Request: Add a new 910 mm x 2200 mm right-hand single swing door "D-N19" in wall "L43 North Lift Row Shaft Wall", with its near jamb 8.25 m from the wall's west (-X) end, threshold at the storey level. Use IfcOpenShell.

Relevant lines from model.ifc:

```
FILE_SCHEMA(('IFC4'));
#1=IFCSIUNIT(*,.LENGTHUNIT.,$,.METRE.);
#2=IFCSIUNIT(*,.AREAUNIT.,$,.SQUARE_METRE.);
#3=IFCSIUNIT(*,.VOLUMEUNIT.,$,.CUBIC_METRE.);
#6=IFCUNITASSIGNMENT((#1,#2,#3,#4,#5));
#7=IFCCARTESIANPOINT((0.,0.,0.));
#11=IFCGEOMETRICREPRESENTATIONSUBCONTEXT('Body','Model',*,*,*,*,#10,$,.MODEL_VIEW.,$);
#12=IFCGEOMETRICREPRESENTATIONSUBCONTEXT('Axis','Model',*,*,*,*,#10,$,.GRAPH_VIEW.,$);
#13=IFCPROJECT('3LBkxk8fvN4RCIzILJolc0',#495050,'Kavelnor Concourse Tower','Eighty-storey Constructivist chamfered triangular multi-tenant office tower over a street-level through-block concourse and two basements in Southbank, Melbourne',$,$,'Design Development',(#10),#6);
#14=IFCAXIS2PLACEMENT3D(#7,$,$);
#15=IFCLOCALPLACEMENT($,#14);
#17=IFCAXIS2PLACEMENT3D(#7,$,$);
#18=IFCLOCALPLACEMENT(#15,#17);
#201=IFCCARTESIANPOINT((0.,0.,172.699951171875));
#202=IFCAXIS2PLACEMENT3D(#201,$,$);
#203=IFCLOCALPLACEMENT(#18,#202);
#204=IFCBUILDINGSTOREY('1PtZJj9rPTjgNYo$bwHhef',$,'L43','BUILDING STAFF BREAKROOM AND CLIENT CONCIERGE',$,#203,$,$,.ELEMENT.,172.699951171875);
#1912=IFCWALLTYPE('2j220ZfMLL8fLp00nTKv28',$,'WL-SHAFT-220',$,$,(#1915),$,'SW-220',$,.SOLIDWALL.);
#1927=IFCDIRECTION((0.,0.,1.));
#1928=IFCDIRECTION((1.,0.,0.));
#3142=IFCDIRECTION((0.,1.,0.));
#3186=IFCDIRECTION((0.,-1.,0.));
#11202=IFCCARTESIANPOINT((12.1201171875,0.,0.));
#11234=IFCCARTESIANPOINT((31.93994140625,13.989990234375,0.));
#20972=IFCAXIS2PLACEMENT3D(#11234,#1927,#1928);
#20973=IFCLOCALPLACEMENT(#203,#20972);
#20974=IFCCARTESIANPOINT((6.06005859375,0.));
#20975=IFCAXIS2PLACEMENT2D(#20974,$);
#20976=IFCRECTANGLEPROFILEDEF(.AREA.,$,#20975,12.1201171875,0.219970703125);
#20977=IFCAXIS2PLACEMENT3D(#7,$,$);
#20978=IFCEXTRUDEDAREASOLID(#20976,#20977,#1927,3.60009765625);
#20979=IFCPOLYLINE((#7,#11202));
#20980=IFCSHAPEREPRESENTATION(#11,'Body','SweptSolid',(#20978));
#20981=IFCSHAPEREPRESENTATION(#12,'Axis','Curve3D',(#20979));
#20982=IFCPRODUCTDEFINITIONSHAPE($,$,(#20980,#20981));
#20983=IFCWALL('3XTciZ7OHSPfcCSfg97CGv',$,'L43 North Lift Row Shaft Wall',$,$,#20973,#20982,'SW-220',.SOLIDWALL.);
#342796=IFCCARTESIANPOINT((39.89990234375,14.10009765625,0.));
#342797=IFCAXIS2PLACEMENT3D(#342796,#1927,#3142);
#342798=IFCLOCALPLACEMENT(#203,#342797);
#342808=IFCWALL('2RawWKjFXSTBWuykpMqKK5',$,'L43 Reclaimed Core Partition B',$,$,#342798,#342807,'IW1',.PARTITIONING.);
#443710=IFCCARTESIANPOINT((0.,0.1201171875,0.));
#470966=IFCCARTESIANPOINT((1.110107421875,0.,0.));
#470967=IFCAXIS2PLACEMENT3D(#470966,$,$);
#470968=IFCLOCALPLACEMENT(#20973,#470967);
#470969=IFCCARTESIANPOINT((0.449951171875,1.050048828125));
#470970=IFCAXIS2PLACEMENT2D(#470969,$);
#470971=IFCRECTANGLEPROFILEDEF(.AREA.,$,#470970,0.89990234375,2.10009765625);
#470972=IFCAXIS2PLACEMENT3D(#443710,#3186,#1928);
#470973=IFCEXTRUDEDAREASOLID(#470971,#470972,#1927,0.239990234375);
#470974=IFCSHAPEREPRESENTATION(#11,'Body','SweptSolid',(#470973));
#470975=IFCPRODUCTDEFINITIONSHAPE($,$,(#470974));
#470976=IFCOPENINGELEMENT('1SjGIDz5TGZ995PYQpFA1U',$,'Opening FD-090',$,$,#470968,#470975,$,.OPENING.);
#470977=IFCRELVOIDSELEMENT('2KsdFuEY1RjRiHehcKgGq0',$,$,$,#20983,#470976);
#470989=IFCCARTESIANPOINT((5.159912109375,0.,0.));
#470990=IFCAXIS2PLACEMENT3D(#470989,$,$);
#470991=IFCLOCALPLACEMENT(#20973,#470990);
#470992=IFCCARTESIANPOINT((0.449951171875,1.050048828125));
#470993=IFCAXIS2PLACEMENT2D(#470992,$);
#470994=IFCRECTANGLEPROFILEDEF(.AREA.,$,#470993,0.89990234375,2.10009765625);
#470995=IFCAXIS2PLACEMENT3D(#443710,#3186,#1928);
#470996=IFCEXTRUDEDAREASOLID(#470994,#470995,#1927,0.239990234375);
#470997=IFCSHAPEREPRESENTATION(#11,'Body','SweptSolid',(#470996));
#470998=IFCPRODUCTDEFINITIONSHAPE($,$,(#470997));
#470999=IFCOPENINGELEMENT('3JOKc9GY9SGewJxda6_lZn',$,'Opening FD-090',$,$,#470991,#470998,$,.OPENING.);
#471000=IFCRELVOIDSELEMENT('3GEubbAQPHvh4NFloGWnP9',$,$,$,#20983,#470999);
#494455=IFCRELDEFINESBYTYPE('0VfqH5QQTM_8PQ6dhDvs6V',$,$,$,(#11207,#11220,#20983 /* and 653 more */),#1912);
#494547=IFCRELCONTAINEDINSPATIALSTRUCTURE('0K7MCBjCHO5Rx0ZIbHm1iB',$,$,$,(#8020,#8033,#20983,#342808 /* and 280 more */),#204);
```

```python
import numpy as np
import ifcopenshell
import ifcopenshell.api.feature
import ifcopenshell.api.geometry
import ifcopenshell.api.root
import ifcopenshell.api.spatial
import ifcopenshell.geom
import ifcopenshell.util.element
import ifcopenshell.util.placement
import ifcopenshell.util.representation
import ifcopenshell.util.shape
import ifcopenshell.util.unit

model = ifcopenshell.open("model.ifc")
unit_scale = ifcopenshell.util.unit.calculate_unit_scale(model)
settings = ifcopenshell.geom.settings()


def volume(element):
    """Net volume in cubic metres, openings subtracted."""
    shape = ifcopenshell.geom.create_shape(settings, element)
    return ifcopenshell.util.shape.get_volume(shape.geometry)


wall = model.by_guid("3XTciZ7OHSPfcCSfg97CGv")
storey = ifcopenshell.util.element.get_container(wall, ifc_class="IfcBuildingStorey")
context = ifcopenshell.util.representation.get_context(model, "Model", "Body", "MODEL_VIEW")
before = volume(wall)

width, height, from_end, sill = 0.91, 2.2, 8.25, 0.0  # metres

# The wall runs along its own X axis, and the end named is its -X end.
wall_shape = ifcopenshell.geom.create_shape(settings, wall)
x, y, z = ifcopenshell.util.shape.get_vertices(wall_shape.geometry).T
start = x.min() + from_end
face, thickness = float(y.min()), float(y.max() - y.min())
wall_matrix = ifcopenshell.util.placement.get_local_placement(wall.ObjectPlacement)
level = ifcopenshell.util.placement.get_local_placement(storey.ObjectPlacement)[2, 3]


def in_wall(x, y):
    """Placement at x, y metres in the wall's axes, at sill height."""
    matrix = wall_matrix.copy()
    matrix[:, 3] = wall_matrix @ np.array([x / unit_scale, y / unit_scale, 0.0, 1.0])
    matrix[2, 3] = level + sill / unit_scale
    return matrix


# Opening: a box that overshoots both wall faces by 50 mm.
opening = ifcopenshell.api.root.create_entity(model, ifc_class="IfcOpeningElement", predefined_type="OPENING")
box = ifcopenshell.api.geometry.add_wall_representation(
    model, context=context, length=width, height=height, thickness=thickness + 0.1
)
ifcopenshell.api.geometry.assign_representation(model, product=opening, representation=box)
ifcopenshell.api.geometry.edit_object_placement(model, product=opening, matrix=in_wall(start, face - 0.05), is_si=False)
ifcopenshell.api.feature.add_feature(model, feature=opening, element=wall)

door = ifcopenshell.api.root.create_entity(model, ifc_class="IfcDoor", name="D-N19", predefined_type="DOOR")
door.OverallWidth, door.OverallHeight = width / unit_scale, height / unit_scale
door.OperationType = "SINGLE_SWING_RIGHT"
body = ifcopenshell.api.geometry.add_door_representation(
    model,
    context=context,
    overall_width=door.OverallWidth,
    overall_height=door.OverallHeight,
    operation_type="SINGLE_SWING_RIGHT",
    lining_properties={"LiningDepth": thickness / unit_scale, "ThresholdDepth": thickness / unit_scale},
)
ifcopenshell.api.geometry.assign_representation(model, product=door, representation=body)
ifcopenshell.api.spatial.assign_container(model, products=[door], relating_structure=storey)
ifcopenshell.api.feature.add_filling(model, opening=opening, element=door)

# The lining spans the wall, so the door starts at the wall face.
ifcopenshell.api.geometry.edit_object_placement(model, product=door, matrix=in_wall(start, face), is_si=False)

after = volume(wall)

print(f"wall volume {before:.3f} -> {after:.3f} m3")

model.write("model_rev.ifc")
```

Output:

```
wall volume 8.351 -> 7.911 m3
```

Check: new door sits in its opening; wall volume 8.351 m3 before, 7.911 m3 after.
